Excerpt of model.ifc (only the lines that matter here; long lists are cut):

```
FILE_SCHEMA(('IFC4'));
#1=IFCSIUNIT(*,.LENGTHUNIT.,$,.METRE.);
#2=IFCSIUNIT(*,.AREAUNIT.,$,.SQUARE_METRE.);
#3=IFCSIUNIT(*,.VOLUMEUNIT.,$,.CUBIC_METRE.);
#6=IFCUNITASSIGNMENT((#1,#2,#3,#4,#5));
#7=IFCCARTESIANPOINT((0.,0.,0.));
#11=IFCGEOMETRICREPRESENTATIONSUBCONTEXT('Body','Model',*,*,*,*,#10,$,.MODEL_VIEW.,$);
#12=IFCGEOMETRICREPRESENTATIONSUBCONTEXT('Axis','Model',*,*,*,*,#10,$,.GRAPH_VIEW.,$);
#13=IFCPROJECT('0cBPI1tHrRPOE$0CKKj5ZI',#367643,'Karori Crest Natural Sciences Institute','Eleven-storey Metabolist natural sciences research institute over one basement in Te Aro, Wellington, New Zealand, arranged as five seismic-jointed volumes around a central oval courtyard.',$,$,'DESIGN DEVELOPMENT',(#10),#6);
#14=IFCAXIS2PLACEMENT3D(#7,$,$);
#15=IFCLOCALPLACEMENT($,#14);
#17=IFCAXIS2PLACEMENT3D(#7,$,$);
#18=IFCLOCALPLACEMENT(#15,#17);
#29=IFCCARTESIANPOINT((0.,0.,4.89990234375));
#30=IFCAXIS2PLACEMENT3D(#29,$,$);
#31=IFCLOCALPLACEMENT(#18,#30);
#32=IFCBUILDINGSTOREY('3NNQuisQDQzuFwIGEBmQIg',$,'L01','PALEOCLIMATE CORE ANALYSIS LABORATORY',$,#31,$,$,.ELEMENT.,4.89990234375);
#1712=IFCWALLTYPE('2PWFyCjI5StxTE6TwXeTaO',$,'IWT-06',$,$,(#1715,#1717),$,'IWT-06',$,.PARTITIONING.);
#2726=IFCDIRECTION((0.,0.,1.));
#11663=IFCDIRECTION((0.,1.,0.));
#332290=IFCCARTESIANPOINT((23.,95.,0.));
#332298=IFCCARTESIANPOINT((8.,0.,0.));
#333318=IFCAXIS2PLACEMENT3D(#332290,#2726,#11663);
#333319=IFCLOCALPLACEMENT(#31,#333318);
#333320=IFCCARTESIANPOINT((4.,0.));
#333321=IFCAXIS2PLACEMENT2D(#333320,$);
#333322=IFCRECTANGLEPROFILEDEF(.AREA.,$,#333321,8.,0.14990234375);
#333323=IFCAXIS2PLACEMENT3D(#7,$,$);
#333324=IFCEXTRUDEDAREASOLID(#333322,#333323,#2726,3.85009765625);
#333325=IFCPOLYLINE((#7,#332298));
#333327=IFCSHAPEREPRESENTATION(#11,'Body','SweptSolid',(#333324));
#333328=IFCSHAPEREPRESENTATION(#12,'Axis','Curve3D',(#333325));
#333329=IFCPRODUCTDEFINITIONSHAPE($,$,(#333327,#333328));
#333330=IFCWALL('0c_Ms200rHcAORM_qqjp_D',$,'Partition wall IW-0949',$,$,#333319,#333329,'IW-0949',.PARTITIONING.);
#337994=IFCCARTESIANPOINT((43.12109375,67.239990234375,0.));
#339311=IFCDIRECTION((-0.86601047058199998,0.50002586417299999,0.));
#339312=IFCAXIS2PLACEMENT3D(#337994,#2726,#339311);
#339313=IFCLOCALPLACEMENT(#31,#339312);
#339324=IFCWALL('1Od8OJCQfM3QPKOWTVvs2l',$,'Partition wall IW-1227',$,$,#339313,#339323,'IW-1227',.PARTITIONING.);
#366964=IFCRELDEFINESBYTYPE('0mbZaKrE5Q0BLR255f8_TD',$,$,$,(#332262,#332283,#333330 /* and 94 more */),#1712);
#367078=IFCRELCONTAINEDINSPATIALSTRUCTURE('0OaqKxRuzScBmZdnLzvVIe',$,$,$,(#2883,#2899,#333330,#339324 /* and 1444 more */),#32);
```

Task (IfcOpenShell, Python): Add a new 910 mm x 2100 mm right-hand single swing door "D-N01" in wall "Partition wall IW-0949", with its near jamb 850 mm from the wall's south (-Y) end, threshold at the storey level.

```python
import numpy as np
import ifcopenshell
import ifcopenshell.api.feature
import ifcopenshell.api.geometry
import ifcopenshell.api.root
import ifcopenshell.api.spatial
import ifcopenshell.geom
import ifcopenshell.util.element
import ifcopenshell.util.placement
import ifcopenshell.util.representation
import ifcopenshell.util.shape
import ifcopenshell.util.unit

model = ifcopenshell.open("model.ifc")
unit_scale = ifcopenshell.util.unit.calculate_unit_scale(model)
settings = ifcopenshell.geom.settings()


def volume(element):
    """Net volume in cubic metres, openings subtracted."""
    shape = ifcopenshell.geom.create_shape(settings, element)
    return ifcopenshell.util.shape.get_volume(shape.geometry)


wall = model.by_id(333330)
storey = ifcopenshell.util.element.get_container(wall, ifc_class="IfcBuildingStorey")
context = ifcopenshell.util.representation.get_context(model, "Model", "Body", "MODEL_VIEW")
before = volume(wall)

width, height, from_end, sill = 0.91, 2.1, 0.85, 0.0  # metres

# The wall runs along its own X axis, and the end named is its -X end.
wall_shape = ifcopenshell.geom.create_shape(settings, wall)
x, y, z = ifcopenshell.util.shape.get_vertices(wall_shape.geometry).T
start = x.min() + from_end
face, thickness = float(y.min()), float(y.max() - y.min())
wall_matrix = ifcopenshell.util.placement.get_local_placement(wall.ObjectPlacement)
level = ifcopenshell.util.placement.get_local_placement(storey.ObjectPlacement)[2, 3]


def in_wall(x, y):
    """Placement at x, y metres in the wall's axes, at sill height."""
    matrix = wall_matrix.copy()
    matrix[:, 3] = wall_matrix @ np.array([x / unit_scale, y / unit_scale, 0.0, 1.0])
    matrix[2, 3] = level + sill / unit_scale
    return matrix


# Opening: a box that overshoots both wall faces by 50 mm.
opening = ifcopenshell.api.root.create_entity(model, ifc_class="IfcOpeningElement", predefined_type="OPENING")
box = ifcopenshell.api.geometry.add_wall_representation(
    model, context=context, length=width, height=height, thickness=thickness + 0.1
)
ifcopenshell.api.geometry.assign_representation(model, product=opening, representation=box)
ifcopenshell.api.geometry.edit_object_placement(model, product=opening, matrix=in_wall(start, face - 0.05), is_si=False)
ifcopenshell.api.feature.add_feature(model, feature=opening, element=wall)

door = ifcopenshell.api.root.create_entity(model, ifc_class="IfcDoor", name="D-N01", predefined_type="DOOR")
door.OverallWidth, door.OverallHeight = width / unit_scale, height / unit_scale
door.OperationType = "SINGLE_SWING_RIGHT"
body = ifcopenshell.api.geometry.add_door_representation(
    model,
    context=context,
    overall_width=door.OverallWidth,
    overall_height=door.OverallHeight,
    operation_type="SINGLE_SWING_RIGHT",
    lining_properties={"LiningDepth": thickness / unit_scale, "ThresholdDepth": thickness / unit_scale},
)
ifcopenshell.api.geometry.assign_representation(model, product=door, representation=body)
ifcopenshell.api.spatial.assign_container(model, products=[door], relating_structure=storey)
ifcopenshell.api.feature.add_filling(model, opening=opening, element=door)

# The lining spans the wall, so the door starts at the wall face.
ifcopenshell.api.geometry.edit_object_placement(model, product=door, matrix=in_wall(start, face), is_si=False)

after = volume(wall)

print(f"wall volume {before:.3f} -> {after:.3f} m3")

model.write("model_v2.ifc")
```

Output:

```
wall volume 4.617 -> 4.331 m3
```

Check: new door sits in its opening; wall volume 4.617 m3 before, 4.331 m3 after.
